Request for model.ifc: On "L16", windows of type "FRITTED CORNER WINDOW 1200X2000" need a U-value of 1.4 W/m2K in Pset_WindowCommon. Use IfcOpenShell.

First a look at what the model holds.

```python
import ifcopenshell
import ifcopenshell.util.element

model = ifcopenshell.open("model.ifc")
print(model.schema)
storey = next(s for s in model.by_type("IfcBuildingStorey") if s.Name == "L16")
windows = [e for e in ifcopenshell.util.element.get_decomposition(storey) if e.is_a("IfcWindow")]
seen = {}
for e in windows:
    element_type = ifcopenshell.util.element.get_type(e)
    key = (element_type.Name if element_type != e and element_type else None, ifcopenshell.util.element.get_pset(e, "Pset_WindowCommon", "ThermalTransmittance"))
    seen[key] = seen.get(key, 0) + 1
for (name, value), count in sorted(seen.items(), key=str):
    print(count, "x", name, "|", value)
```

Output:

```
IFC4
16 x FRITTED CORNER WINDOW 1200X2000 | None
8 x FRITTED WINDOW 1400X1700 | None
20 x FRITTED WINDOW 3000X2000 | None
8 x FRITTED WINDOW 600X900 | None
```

```python
import ifcopenshell
import ifcopenshell.api.pset
import ifcopenshell.util.element

model = ifcopenshell.open("model.ifc")

storey = next(s for s in model.by_type("IfcBuildingStorey") if s.Name == "L16")
windows = [e for e in ifcopenshell.util.element.get_decomposition(storey) if e.is_a("IfcWindow")]

count = 0
for e in windows:
    element_type = ifcopenshell.util.element.get_type(e)
    if element_type in (None, e) or element_type.Name != "FRITTED CORNER WINDOW 1200X2000":
        continue
    found = ifcopenshell.util.element.get_pset(e, "Pset_WindowCommon", should_inherit=False)
    if found:
        pset = model.by_id(found["id"])
        if len(ifcopenshell.util.element.get_elements_by_pset(pset)) > 1:
            pset = ifcopenshell.api.pset.unshare_pset(model, products=[e], pset=pset)[0]
    else:
        pset = ifcopenshell.api.pset.add_pset(model, product=e, name="Pset_WindowCommon")
    ifcopenshell.api.pset.edit_pset(model, pset=pset, properties={"ThermalTransmittance": 1.4})
    count += 1

print(count, "windows updated")

model.write("model_updated.ifc")
```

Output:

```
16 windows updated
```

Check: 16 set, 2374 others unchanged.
